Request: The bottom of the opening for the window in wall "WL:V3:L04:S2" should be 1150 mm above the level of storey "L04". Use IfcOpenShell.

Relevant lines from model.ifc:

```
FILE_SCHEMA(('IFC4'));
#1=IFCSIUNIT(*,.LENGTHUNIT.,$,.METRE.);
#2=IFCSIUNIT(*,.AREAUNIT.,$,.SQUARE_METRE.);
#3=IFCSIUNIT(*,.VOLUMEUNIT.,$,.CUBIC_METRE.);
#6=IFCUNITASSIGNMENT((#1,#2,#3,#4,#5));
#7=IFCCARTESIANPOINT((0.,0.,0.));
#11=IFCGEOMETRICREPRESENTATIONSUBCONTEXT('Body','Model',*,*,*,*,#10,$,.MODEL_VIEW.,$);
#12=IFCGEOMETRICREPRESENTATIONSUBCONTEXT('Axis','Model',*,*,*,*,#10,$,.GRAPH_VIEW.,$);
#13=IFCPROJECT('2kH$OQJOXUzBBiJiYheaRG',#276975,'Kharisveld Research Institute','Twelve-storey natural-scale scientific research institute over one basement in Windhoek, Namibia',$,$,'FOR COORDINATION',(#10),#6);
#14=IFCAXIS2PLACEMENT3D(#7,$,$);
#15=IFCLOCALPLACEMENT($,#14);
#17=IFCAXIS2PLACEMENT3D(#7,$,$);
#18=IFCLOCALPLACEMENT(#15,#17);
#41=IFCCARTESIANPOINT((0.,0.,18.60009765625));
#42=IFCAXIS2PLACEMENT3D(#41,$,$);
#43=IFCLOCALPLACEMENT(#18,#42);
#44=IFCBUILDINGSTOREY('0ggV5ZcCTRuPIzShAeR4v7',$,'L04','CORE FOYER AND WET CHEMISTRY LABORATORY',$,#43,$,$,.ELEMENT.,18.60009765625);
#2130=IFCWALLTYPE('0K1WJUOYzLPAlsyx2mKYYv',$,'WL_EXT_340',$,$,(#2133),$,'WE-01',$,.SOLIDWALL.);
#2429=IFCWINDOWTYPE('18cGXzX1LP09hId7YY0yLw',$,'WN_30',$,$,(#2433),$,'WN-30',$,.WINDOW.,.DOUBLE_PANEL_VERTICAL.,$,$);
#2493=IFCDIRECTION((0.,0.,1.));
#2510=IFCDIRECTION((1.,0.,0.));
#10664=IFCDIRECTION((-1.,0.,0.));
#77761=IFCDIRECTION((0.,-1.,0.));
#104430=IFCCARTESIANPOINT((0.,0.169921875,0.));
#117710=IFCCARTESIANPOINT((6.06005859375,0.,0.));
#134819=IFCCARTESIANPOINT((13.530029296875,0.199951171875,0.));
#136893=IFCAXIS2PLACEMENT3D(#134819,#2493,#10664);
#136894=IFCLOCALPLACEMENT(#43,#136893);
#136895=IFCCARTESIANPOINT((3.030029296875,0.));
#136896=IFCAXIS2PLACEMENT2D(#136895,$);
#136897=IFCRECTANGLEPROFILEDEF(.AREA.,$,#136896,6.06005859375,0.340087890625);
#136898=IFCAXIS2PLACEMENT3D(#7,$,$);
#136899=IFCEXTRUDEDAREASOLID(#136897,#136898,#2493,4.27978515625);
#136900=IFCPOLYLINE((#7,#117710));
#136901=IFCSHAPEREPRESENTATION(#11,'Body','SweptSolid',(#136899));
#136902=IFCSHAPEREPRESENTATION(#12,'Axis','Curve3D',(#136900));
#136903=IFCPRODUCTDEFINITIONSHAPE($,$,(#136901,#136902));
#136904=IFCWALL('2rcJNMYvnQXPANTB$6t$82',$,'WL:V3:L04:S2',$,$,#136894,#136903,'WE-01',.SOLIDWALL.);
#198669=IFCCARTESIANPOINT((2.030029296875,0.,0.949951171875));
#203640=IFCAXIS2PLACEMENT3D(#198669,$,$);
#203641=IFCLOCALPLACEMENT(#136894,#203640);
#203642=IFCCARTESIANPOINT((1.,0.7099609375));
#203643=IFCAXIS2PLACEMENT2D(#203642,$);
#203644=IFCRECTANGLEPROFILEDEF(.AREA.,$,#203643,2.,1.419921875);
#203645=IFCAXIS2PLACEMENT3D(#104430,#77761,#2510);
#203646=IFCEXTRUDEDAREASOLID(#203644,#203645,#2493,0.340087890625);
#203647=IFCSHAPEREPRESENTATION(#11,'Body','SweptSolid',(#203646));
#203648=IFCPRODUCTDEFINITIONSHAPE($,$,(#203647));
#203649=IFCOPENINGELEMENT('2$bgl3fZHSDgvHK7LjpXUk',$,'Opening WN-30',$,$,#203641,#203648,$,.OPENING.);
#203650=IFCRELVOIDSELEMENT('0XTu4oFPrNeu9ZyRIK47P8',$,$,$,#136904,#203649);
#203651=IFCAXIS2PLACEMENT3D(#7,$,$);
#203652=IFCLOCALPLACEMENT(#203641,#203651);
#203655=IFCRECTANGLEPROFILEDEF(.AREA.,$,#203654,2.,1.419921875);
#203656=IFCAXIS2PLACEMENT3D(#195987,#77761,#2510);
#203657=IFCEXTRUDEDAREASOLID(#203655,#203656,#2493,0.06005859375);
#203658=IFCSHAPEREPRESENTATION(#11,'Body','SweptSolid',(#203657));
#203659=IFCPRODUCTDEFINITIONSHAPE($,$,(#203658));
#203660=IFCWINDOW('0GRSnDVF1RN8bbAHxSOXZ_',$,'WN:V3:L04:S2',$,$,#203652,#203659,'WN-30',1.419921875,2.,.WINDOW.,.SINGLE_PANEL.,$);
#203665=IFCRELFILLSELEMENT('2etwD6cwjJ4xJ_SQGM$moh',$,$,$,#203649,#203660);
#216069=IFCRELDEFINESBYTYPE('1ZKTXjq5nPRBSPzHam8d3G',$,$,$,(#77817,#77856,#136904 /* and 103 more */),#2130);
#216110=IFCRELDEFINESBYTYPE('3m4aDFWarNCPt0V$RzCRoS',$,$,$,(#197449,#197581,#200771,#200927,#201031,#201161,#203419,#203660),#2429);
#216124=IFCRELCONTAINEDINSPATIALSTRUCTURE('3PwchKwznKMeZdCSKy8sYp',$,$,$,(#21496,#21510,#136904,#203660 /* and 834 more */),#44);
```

```python
import numpy as np
import ifcopenshell
import ifcopenshell.api.geometry
import ifcopenshell.geom
import ifcopenshell.util.element
import ifcopenshell.util.placement
import ifcopenshell.util.shape
import ifcopenshell.util.unit

model = ifcopenshell.open("model.ifc")
unit_scale = ifcopenshell.util.unit.calculate_unit_scale(model)

window = model.by_guid("0GRSnDVF1RN8bbAHxSOXZ_")
opening = window.FillsVoids[0].RelatingOpeningElement
storey = ifcopenshell.util.element.get_container(window, ifc_class="IfcBuildingStorey")
level = ifcopenshell.util.placement.get_local_placement(storey.ObjectPlacement)[2, 3]

# The opening's origin need not be at the sill, so measure its lowest point.
shape = ifcopenshell.geom.create_shape(ifcopenshell.geom.settings(), opening)
bottom = ifcopenshell.util.shape.get_shape_bottom_elevation(shape, shape.geometry) / unit_scale
dz = level + 1.15 / unit_scale - bottom

shift = np.array([0.0, 0.0, dz])
# The window is placed relative to its opening, so it follows when the opening moves.
matrix = ifcopenshell.util.placement.get_local_placement(opening.ObjectPlacement)
matrix[:3, 3] += shift
ifcopenshell.api.geometry.edit_object_placement(
    model, product=opening, matrix=matrix, is_si=False, should_transform_children=True
)

print(f"moved by {dz * unit_scale:+.3f} m")

model.write("model_edited.ifc")
```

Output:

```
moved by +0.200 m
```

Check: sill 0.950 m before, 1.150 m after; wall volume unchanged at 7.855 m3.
